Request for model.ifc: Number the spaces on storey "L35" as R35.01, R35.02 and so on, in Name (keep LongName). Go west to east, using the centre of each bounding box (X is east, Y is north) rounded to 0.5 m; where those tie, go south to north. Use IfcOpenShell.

First a look at what the model holds.

```python
import ifcopenshell
import ifcopenshell.util.element
import ifcopenshell.util.placement

model = ifcopenshell.open("model.ifc")
print(model.schema)
storey = next(s for s in model.by_type("IfcBuildingStorey") if s.Name == "L35")
spaces = [e for e in ifcopenshell.util.element.get_decomposition(storey) if e.is_a("IfcSpace")]
for e in sorted(spaces, key=lambda e: e.id()):
    origin = ifcopenshell.util.placement.get_local_placement(e.ObjectPlacement)[:3, 3]
    print(e.id(), e.Name, e.LongName, origin.round(2) + 0.0, sep=" | ")
```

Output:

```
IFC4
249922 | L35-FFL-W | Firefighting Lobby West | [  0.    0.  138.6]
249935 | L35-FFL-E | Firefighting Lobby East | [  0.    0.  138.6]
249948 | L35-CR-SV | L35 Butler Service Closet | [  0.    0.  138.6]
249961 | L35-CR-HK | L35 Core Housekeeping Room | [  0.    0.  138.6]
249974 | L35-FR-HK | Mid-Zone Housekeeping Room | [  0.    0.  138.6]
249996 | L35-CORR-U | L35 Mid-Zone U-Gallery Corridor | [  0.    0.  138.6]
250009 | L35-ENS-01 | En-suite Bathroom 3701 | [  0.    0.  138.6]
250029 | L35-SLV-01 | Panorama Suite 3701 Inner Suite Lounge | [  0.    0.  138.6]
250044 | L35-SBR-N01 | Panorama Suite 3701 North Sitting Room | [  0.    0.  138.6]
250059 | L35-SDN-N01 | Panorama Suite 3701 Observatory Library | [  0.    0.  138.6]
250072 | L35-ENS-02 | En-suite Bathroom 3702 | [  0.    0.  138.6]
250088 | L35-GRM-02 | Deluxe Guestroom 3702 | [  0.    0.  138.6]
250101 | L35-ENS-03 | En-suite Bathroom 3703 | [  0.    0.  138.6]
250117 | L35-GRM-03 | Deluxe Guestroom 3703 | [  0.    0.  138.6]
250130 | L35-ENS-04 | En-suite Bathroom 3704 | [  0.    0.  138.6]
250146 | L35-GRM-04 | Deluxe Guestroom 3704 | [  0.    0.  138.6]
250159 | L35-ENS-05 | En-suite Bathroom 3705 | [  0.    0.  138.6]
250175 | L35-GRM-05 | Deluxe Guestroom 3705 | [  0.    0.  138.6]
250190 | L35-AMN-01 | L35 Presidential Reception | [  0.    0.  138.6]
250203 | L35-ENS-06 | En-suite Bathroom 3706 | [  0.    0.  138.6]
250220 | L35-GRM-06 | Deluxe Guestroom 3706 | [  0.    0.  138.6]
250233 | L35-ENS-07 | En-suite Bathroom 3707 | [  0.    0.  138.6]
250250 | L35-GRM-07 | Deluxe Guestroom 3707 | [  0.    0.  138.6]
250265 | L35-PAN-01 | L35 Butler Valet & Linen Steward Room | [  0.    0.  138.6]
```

```python
import ifcopenshell
import ifcopenshell.geom
import ifcopenshell.util.element
import ifcopenshell.util.shape

model = ifcopenshell.open("model.ifc")
settings = ifcopenshell.geom.settings()
settings.set("use-world-coords", True)


def centre(element):
    shape = ifcopenshell.geom.create_shape(settings, element)
    return ifcopenshell.util.shape.get_bbox_centroid(shape.geometry)


storey = next(s for s in model.by_type("IfcBuildingStorey") if s.Name == "L35")
spaces = [e for e in ifcopenshell.util.element.get_decomposition(storey) if e.is_a("IfcSpace")]

# Insertion points can sit at a corner or the storey origin, so sort by the geometry (in metres).
centres = {e: centre(e) for e in spaces}
spaces.sort(key=lambda e: (round(centres[e][0] / 0.5), centres[e][1]))

for i, e in enumerate(spaces, start=1):
    number = f"R35.{i:02d}"
    e.Name = number
    print(e.id(), number)

model.write("model_edited.ifc")
```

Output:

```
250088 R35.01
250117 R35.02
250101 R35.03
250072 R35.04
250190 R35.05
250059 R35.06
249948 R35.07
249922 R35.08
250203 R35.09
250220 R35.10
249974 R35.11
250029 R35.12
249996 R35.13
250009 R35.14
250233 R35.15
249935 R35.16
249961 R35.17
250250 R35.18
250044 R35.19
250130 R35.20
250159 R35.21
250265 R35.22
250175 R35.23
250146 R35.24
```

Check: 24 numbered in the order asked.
